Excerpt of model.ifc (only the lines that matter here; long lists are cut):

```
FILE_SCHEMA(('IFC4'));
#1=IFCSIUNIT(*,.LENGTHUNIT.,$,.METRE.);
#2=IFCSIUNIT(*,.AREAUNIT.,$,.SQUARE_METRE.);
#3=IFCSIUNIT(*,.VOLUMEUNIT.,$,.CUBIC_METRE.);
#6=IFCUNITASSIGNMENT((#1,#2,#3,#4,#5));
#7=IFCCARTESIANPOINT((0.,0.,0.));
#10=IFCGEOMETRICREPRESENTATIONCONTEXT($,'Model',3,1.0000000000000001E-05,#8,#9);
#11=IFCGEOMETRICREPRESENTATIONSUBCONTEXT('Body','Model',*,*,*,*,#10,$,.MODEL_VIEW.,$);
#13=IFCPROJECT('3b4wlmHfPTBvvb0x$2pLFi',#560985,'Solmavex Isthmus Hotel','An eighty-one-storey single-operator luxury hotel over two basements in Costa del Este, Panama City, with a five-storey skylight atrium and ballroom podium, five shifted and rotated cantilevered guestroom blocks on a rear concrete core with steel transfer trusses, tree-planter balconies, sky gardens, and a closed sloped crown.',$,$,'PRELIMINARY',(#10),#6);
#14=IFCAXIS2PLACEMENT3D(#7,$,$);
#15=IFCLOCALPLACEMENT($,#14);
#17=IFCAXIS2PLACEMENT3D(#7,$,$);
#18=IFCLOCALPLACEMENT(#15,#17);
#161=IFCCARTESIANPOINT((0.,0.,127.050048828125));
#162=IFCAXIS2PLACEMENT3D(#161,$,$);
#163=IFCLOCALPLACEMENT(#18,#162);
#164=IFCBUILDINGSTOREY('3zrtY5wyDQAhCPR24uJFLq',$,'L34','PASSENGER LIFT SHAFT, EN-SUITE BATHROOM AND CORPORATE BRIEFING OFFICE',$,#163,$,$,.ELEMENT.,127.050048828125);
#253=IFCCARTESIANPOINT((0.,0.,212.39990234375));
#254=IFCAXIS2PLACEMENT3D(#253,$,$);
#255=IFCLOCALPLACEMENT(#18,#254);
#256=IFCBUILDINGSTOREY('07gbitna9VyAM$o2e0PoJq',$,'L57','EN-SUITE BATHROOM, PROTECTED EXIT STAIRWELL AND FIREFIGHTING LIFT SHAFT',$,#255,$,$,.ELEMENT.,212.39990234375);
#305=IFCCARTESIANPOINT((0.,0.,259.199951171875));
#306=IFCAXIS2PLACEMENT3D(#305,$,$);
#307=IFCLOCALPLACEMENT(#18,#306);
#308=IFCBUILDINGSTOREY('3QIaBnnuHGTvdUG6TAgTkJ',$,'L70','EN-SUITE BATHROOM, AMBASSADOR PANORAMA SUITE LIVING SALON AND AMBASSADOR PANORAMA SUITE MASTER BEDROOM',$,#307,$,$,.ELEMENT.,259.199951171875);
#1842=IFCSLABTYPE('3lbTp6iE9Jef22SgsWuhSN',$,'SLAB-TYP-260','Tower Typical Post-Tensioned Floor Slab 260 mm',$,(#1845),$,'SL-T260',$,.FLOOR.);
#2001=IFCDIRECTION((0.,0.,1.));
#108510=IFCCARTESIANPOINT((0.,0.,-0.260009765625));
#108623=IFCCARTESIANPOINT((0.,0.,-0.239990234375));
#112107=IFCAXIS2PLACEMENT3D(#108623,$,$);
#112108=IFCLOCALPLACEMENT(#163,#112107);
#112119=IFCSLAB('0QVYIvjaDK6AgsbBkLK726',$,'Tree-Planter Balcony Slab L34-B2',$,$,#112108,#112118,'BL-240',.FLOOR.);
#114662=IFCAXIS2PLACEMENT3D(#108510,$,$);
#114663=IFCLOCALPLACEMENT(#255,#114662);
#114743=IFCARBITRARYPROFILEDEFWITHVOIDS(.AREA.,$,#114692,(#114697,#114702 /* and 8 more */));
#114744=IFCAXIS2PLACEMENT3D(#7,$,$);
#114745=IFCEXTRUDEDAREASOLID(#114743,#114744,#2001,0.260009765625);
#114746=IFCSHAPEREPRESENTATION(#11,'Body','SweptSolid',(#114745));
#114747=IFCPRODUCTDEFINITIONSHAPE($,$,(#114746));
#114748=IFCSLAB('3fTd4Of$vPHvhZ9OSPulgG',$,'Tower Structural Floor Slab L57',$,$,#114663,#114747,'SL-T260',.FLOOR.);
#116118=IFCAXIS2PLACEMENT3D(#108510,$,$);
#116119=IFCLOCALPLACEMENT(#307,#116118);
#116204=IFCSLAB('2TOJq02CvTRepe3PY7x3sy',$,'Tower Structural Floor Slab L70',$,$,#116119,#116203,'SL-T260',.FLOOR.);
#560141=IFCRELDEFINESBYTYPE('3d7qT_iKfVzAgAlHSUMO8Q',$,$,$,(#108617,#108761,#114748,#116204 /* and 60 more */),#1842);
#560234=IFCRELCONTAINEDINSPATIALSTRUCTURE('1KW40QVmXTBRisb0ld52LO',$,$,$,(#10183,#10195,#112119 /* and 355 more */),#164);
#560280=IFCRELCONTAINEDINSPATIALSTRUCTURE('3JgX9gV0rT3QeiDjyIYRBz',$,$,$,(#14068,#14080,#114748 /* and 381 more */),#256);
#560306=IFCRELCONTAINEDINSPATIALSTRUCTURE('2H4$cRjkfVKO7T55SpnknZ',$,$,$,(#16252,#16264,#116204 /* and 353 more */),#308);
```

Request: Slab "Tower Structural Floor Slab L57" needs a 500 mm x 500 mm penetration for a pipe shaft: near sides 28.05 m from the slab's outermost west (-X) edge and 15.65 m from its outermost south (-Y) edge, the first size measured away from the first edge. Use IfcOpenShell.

```python
import numpy as np
import ifcopenshell
import ifcopenshell.api.feature
import ifcopenshell.api.geometry
import ifcopenshell.api.root
import ifcopenshell.geom
import ifcopenshell.util.placement
import ifcopenshell.util.representation
import ifcopenshell.util.shape
import ifcopenshell.util.unit

model = ifcopenshell.open("model.ifc")
unit_scale = ifcopenshell.util.unit.calculate_unit_scale(model)
settings = ifcopenshell.geom.settings()


def volume(element):
    """Net volume in cubic metres, openings subtracted."""
    shape = ifcopenshell.geom.create_shape(settings, element)
    return ifcopenshell.util.shape.get_volume(shape.geometry)


slab = model.by_id(114748)
before = volume(slab)

# Extent in the slab's own axes, in metres. The edges named are its -X and -Y sides.
slab_shape = ifcopenshell.geom.create_shape(settings, slab)
vertices = ifcopenshell.util.shape.get_vertices(slab_shape.geometry)
x_min, y_min, bottom = vertices.min(axis=0)
top = vertices[:, 2].max()

opening = ifcopenshell.api.root.create_entity(model, ifc_class="IfcOpeningElement", name="Pipe shaft opening", predefined_type="OPENING")
context = ifcopenshell.util.representation.get_context(model, "Model", "Body", "MODEL_VIEW")
width, depth = 0.5, 0.5
outline = [(0.0, 0.0), (width, 0.0), (width, depth), (0.0, depth), (0.0, 0.0)]
# Overshoot both faces by 50 mm so the cut is clean.
shape = ifcopenshell.api.geometry.add_slab_representation(
    model, context=context, depth=top - bottom + 0.1, polyline=outline
)
ifcopenshell.api.geometry.assign_representation(model, product=opening, representation=shape)

matrix = ifcopenshell.util.placement.get_local_placement(slab.ObjectPlacement)
matrix[:, 3] = matrix @ np.append(np.array([x_min + 28.05, y_min + 15.65, bottom - 0.05]) / unit_scale, 1.0)
ifcopenshell.api.geometry.edit_object_placement(model, product=opening, matrix=matrix, is_si=False)
ifcopenshell.api.feature.add_feature(model, feature=opening, element=slab)

after = volume(slab)

print(f"slab volume {before:.3f} -> {after:.3f} m3")

model.write("model_edited.ifc")
```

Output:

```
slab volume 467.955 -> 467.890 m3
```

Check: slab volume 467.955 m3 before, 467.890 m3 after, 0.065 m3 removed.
